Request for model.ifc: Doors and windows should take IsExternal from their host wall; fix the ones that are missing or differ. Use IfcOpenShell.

First a look at what the model holds.

```python
import ifcopenshell
import ifcopenshell.util.element

model = ifcopenshell.open("model.ifc")
print(model.schema)
seen = {}
for e in model.by_type("IfcDoor") + model.by_type("IfcWindow"):
    if not e.FillsVoids:
        continue
    host = e.FillsVoids[0].RelatingOpeningElement.VoidsElements[0].RelatingBuildingElement
    own = ifcopenshell.util.element.get_pset(e, f"Pset_{e.is_a()[3:].removesuffix('StandardCase')}Common", "IsExternal")
    wall = ifcopenshell.util.element.get_pset(host, "Pset_WallCommon", "IsExternal")
    seen[e.is_a(), own, wall] = seen.get((e.is_a(), own, wall), 0) + 1
for (cls, own, wall), count in sorted(seen.items(), key=str):
    print(count, cls, "IsExternal:", own, "| host wall:", wall)
```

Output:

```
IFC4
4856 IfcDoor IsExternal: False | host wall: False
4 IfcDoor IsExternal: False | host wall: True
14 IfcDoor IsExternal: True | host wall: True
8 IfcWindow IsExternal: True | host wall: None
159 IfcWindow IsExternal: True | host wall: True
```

```python
import ifcopenshell
import ifcopenshell.api.pset
import ifcopenshell.util.element

model = ifcopenshell.open("model.ifc")

count = 0
for ifc_class, pset_name in (("IfcDoor", "Pset_DoorCommon"), ("IfcWindow", "Pset_WindowCommon")):
    for e in model.by_type(ifc_class):
        if not e.FillsVoids:
            continue
        host = e.FillsVoids[0].RelatingOpeningElement.VoidsElements[0].RelatingBuildingElement
        external = ifcopenshell.util.element.get_pset(host, "Pset_WallCommon", "IsExternal")
        if external is None or ifcopenshell.util.element.get_pset(e, pset_name, "IsExternal") == external:
            continue
        found = ifcopenshell.util.element.get_pset(e, pset_name, should_inherit=False)
        if found:
            pset = model.by_id(found["id"])
            if len(ifcopenshell.util.element.get_elements_by_pset(pset)) > 1:
                pset = ifcopenshell.api.pset.unshare_pset(model, products=[e], pset=pset)[0]
        else:
            pset = ifcopenshell.api.pset.add_pset(model, product=e, name=pset_name)
        ifcopenshell.api.pset.edit_pset(model, pset=pset, properties={"IsExternal": external})
        count += 1

print(count, "updated")

model.write("model_updated.ifc")
```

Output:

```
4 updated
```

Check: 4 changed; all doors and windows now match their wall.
